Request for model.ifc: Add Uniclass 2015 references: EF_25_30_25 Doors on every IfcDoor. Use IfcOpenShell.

First a look at what the model holds.

```python
import ifcopenshell

model = ifcopenshell.open("model.ifc")
print(model.schema)
print("classifications:", [c.Name for c in model.by_type("IfcClassification")])
for ifc_class in ("IfcDoor", "IfcRoof", "IfcStair", "IfcWall", "IfcWindow"):
    print(ifc_class, len(model.by_type(ifc_class)))
```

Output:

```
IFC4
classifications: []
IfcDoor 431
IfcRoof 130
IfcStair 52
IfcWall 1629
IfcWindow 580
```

```python
import ifcopenshell
import ifcopenshell.api.classification

model = ifcopenshell.open("model.ifc")

system = ifcopenshell.api.classification.add_classification(model, classification="Uniclass 2015")

codes = {
    "IfcDoor": ("EF_25_30_25", "Doors"),
}
for ifc_class, (code, name) in codes.items():
    products = model.by_type(ifc_class)
    ifcopenshell.api.classification.add_reference(
        model, products=products, classification=system, identification=code, name=name
    )
    print(code, len(products))

model.write("model-out.ifc")
```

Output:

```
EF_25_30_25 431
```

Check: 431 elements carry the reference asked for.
